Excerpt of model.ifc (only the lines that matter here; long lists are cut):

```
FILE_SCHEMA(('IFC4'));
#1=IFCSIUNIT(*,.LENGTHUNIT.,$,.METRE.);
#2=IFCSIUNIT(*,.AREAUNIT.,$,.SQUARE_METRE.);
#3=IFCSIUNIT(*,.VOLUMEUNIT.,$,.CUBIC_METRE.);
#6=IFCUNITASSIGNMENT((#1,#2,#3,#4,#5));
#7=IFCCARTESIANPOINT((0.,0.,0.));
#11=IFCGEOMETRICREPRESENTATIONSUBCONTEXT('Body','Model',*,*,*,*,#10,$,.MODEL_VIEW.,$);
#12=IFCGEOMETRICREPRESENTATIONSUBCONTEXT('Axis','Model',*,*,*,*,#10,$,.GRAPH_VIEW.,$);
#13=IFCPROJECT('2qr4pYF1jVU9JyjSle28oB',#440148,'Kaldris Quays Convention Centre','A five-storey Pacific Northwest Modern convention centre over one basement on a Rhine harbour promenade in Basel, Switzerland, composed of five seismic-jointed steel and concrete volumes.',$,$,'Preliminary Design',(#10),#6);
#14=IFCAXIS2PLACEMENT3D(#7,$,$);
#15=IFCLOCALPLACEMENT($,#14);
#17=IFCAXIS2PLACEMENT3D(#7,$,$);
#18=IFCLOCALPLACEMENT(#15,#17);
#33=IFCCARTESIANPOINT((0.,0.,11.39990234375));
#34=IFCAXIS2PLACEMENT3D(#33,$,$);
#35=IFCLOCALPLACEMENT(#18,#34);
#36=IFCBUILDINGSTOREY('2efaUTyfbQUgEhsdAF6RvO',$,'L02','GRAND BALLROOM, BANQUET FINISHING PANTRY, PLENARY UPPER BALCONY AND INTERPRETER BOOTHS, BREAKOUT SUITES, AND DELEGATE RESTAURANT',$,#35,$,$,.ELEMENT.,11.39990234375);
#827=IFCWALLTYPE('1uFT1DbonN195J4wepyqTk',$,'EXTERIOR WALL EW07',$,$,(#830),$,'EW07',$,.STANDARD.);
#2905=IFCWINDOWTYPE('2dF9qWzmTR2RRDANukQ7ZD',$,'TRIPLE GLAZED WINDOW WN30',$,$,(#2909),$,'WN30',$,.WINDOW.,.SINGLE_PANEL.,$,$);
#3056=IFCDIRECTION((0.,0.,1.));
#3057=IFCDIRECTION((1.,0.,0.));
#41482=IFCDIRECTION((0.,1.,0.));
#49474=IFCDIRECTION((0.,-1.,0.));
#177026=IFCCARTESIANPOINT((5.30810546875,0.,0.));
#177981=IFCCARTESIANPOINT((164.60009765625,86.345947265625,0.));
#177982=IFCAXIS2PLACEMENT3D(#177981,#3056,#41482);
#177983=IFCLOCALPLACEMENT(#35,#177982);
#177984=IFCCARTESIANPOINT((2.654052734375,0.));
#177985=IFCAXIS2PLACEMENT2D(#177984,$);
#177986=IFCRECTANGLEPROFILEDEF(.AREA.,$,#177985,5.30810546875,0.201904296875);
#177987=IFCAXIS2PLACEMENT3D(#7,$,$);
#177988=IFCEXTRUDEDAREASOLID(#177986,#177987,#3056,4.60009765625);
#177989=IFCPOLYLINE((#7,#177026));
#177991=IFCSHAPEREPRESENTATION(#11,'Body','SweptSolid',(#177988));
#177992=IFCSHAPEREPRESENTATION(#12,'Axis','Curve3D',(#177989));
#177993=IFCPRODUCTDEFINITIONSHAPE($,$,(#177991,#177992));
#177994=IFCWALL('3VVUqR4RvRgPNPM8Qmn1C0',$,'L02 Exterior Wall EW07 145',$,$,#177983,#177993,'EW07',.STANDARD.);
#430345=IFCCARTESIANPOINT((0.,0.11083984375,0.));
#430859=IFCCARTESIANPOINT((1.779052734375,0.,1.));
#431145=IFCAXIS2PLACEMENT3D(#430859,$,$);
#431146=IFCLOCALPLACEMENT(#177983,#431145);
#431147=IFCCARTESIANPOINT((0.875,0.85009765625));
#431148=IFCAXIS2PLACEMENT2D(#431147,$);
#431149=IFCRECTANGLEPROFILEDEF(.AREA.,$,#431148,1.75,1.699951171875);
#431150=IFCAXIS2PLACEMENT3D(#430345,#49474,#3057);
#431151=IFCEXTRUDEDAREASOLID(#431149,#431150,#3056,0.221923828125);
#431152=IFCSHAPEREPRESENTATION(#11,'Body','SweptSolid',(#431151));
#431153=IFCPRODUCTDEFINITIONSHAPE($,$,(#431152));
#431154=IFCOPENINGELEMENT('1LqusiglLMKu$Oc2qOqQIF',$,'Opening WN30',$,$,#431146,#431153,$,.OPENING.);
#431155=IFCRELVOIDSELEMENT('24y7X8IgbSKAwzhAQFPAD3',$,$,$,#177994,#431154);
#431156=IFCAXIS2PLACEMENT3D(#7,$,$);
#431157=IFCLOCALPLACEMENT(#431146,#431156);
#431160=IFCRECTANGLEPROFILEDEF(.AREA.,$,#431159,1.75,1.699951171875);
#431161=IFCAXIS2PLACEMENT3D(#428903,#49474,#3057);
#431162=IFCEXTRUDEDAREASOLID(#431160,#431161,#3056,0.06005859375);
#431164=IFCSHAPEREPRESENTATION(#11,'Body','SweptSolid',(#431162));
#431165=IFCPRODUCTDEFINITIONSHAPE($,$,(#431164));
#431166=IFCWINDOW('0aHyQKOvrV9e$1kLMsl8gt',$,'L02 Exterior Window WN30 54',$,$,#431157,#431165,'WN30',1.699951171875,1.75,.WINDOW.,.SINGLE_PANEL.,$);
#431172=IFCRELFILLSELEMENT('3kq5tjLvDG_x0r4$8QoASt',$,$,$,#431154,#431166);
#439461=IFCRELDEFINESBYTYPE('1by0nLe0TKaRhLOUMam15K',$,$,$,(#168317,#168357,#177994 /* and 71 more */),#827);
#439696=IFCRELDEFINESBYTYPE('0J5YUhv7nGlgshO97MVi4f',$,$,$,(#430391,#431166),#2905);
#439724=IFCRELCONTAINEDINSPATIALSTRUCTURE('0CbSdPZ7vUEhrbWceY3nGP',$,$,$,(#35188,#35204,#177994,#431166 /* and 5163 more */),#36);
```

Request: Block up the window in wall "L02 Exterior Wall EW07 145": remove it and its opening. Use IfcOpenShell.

```python
import ifcopenshell
import ifcopenshell.api.feature
import ifcopenshell.api.root
import ifcopenshell.geom
import ifcopenshell.util.shape

model = ifcopenshell.open("model.ifc")
settings = ifcopenshell.geom.settings()


def volume(element):
    """Net volume in cubic metres, openings subtracted."""
    shape = ifcopenshell.geom.create_shape(settings, element)
    return ifcopenshell.util.shape.get_volume(shape.geometry)


window = model.by_id(431166)
opening = window.FillsVoids[0].RelatingOpeningElement
wall = opening.VoidsElements[0].RelatingBuildingElement
before = volume(wall)

ifcopenshell.api.root.remove_product(model, product=window)
ifcopenshell.api.feature.remove_feature(model, feature=opening)

after = volume(wall)

print(f"wall volume {before:.3f} -> {after:.3f} m3")

model.write("model_rev.ifc")
```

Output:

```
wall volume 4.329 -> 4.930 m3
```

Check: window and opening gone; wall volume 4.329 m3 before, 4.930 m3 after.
